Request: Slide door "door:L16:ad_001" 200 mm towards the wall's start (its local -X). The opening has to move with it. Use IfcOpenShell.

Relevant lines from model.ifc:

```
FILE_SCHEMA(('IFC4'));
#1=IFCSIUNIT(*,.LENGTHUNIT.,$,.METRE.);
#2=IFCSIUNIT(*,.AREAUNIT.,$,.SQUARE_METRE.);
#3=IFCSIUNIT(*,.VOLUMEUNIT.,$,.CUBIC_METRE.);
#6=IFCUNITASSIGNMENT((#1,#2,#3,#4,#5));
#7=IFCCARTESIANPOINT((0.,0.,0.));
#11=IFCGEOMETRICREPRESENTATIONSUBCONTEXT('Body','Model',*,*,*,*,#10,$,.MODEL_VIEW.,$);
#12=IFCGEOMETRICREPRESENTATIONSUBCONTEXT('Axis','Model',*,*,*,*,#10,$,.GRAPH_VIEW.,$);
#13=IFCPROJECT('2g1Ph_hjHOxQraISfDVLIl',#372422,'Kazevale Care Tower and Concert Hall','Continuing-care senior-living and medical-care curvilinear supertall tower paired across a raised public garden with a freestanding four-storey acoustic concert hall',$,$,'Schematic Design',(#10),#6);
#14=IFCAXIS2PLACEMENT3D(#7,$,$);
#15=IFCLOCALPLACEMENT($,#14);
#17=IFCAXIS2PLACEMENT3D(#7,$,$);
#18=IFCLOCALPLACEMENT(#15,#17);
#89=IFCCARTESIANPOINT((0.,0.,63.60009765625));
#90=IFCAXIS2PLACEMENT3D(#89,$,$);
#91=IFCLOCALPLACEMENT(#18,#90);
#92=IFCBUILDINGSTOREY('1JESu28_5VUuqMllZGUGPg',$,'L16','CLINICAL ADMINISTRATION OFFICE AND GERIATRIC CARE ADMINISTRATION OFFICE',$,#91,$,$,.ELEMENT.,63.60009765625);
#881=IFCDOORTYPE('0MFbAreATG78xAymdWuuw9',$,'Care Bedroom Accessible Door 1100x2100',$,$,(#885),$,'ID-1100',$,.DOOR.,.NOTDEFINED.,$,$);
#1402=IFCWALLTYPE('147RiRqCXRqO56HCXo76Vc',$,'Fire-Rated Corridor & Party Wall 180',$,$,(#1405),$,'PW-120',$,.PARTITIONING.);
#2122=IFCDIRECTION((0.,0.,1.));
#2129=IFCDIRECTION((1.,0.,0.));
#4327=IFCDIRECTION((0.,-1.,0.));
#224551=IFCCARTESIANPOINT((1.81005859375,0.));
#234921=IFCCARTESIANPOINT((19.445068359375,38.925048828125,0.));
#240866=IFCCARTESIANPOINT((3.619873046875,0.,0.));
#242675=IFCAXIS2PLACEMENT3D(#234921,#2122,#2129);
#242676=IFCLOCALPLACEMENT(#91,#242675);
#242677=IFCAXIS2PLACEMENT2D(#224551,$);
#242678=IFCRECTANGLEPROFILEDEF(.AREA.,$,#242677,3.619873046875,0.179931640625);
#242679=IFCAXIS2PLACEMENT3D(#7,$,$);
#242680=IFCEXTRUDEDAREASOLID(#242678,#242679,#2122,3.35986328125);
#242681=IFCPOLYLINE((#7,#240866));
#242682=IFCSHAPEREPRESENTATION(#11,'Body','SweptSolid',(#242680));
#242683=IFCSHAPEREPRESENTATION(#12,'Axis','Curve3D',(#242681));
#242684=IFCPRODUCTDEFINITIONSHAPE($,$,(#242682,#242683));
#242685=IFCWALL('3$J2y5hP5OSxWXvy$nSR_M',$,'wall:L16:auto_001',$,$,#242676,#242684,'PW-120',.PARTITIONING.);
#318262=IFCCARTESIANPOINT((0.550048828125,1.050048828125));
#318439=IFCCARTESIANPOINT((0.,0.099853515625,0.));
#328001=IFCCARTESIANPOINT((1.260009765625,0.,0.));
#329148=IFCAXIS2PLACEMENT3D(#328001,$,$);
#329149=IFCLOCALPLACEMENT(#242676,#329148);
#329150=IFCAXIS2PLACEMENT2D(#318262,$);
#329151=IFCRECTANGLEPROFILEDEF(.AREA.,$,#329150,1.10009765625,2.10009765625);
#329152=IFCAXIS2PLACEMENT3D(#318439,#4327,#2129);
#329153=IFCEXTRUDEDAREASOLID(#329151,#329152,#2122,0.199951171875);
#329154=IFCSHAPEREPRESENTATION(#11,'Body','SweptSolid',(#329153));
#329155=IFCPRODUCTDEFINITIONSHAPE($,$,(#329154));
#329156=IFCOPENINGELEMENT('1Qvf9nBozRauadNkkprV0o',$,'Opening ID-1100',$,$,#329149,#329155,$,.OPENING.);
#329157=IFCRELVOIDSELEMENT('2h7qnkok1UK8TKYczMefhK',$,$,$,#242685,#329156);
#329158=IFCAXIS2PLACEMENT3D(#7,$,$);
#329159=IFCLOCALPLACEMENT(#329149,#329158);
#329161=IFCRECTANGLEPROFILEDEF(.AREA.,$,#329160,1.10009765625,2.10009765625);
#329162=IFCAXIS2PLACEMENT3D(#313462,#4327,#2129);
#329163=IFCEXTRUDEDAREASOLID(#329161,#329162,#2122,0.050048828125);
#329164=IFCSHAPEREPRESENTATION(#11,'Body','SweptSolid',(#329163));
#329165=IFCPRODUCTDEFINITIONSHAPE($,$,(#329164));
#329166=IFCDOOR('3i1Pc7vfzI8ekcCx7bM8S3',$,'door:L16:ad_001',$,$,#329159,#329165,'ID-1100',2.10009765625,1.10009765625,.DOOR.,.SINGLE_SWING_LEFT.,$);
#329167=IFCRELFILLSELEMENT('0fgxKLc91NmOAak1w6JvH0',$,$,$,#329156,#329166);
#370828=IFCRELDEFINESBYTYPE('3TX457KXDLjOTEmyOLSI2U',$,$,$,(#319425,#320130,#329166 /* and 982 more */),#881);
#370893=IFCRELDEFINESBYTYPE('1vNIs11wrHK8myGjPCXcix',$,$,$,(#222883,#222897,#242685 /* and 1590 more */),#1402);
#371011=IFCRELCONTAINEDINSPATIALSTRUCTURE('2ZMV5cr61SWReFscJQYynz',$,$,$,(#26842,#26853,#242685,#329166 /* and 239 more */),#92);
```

```python
import ifcopenshell
import ifcopenshell.api.geometry
import ifcopenshell.util.placement
import ifcopenshell.util.unit

model = ifcopenshell.open("model.ifc")
unit_scale = ifcopenshell.util.unit.calculate_unit_scale(model)

door = model.by_guid("3i1Pc7vfzI8ekcCx7bM8S3")
opening = door.FillsVoids[0].RelatingOpeningElement
wall = opening.VoidsElements[0].RelatingBuildingElement

wall_matrix = ifcopenshell.util.placement.get_local_placement(wall.ObjectPlacement)
shift = wall_matrix[:3, 0] * -0.2 / unit_scale
before = ifcopenshell.util.placement.get_local_placement(door.ObjectPlacement)[:3, 3].copy()

# The door is placed relative to its opening, so it follows when the opening moves.
matrix = ifcopenshell.util.placement.get_local_placement(opening.ObjectPlacement)
matrix[:3, 3] += shift
ifcopenshell.api.geometry.edit_object_placement(
    model, product=opening, matrix=matrix, is_si=False, should_transform_children=True
)

after = ifcopenshell.util.placement.get_local_placement(door.ObjectPlacement)[:3, 3]
print("door moved by", (after - before).round(3) + 0.0)

model.write("model_rev.ifc")
```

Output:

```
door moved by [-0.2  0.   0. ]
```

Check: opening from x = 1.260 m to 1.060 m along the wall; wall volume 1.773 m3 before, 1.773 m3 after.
